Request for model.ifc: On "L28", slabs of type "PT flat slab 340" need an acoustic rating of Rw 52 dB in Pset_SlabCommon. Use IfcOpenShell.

First a look at what the model holds.

```python
import ifcopenshell
import ifcopenshell.util.element

model = ifcopenshell.open("model.ifc")
print(model.schema)
storey = next(s for s in model.by_type("IfcBuildingStorey") if s.Name == "L28")
slabs = [e for e in ifcopenshell.util.element.get_decomposition(storey) if e.is_a("IfcSlab")]
seen = {}
for e in slabs:
    element_type = ifcopenshell.util.element.get_type(e)
    key = (element_type.Name if element_type != e and element_type else None, ifcopenshell.util.element.get_pset(e, "Pset_SlabCommon", "AcousticRating"))
    seen[key] = seen.get(key, 0) + 1
for (name, value), count in sorted(seen.items(), key=str):
    print(count, "x", name, "|", value)
```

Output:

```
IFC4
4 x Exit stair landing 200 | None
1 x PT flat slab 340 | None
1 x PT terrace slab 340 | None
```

```python
import ifcopenshell
import ifcopenshell.api.pset
import ifcopenshell.util.element

model = ifcopenshell.open("model.ifc")

storey = next(s for s in model.by_type("IfcBuildingStorey") if s.Name == "L28")
slabs = [e for e in ifcopenshell.util.element.get_decomposition(storey) if e.is_a("IfcSlab")]

count = 0
for e in slabs:
    element_type = ifcopenshell.util.element.get_type(e)
    if element_type in (None, e) or element_type.Name != "PT flat slab 340":
        continue
    found = ifcopenshell.util.element.get_pset(e, "Pset_SlabCommon", should_inherit=False)
    if found:
        pset = model.by_id(found["id"])
        if len(ifcopenshell.util.element.get_elements_by_pset(pset)) > 1:
            pset = ifcopenshell.api.pset.unshare_pset(model, products=[e], pset=pset)[0]
    else:
        pset = ifcopenshell.api.pset.add_pset(model, product=e, name="Pset_SlabCommon")
    ifcopenshell.api.pset.edit_pset(model, pset=pset, properties={"AcousticRating": "Rw 52 dB"})
    count += 1

print(count, "slabs updated")

model.write("model_rev.ifc")
```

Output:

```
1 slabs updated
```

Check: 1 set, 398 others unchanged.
